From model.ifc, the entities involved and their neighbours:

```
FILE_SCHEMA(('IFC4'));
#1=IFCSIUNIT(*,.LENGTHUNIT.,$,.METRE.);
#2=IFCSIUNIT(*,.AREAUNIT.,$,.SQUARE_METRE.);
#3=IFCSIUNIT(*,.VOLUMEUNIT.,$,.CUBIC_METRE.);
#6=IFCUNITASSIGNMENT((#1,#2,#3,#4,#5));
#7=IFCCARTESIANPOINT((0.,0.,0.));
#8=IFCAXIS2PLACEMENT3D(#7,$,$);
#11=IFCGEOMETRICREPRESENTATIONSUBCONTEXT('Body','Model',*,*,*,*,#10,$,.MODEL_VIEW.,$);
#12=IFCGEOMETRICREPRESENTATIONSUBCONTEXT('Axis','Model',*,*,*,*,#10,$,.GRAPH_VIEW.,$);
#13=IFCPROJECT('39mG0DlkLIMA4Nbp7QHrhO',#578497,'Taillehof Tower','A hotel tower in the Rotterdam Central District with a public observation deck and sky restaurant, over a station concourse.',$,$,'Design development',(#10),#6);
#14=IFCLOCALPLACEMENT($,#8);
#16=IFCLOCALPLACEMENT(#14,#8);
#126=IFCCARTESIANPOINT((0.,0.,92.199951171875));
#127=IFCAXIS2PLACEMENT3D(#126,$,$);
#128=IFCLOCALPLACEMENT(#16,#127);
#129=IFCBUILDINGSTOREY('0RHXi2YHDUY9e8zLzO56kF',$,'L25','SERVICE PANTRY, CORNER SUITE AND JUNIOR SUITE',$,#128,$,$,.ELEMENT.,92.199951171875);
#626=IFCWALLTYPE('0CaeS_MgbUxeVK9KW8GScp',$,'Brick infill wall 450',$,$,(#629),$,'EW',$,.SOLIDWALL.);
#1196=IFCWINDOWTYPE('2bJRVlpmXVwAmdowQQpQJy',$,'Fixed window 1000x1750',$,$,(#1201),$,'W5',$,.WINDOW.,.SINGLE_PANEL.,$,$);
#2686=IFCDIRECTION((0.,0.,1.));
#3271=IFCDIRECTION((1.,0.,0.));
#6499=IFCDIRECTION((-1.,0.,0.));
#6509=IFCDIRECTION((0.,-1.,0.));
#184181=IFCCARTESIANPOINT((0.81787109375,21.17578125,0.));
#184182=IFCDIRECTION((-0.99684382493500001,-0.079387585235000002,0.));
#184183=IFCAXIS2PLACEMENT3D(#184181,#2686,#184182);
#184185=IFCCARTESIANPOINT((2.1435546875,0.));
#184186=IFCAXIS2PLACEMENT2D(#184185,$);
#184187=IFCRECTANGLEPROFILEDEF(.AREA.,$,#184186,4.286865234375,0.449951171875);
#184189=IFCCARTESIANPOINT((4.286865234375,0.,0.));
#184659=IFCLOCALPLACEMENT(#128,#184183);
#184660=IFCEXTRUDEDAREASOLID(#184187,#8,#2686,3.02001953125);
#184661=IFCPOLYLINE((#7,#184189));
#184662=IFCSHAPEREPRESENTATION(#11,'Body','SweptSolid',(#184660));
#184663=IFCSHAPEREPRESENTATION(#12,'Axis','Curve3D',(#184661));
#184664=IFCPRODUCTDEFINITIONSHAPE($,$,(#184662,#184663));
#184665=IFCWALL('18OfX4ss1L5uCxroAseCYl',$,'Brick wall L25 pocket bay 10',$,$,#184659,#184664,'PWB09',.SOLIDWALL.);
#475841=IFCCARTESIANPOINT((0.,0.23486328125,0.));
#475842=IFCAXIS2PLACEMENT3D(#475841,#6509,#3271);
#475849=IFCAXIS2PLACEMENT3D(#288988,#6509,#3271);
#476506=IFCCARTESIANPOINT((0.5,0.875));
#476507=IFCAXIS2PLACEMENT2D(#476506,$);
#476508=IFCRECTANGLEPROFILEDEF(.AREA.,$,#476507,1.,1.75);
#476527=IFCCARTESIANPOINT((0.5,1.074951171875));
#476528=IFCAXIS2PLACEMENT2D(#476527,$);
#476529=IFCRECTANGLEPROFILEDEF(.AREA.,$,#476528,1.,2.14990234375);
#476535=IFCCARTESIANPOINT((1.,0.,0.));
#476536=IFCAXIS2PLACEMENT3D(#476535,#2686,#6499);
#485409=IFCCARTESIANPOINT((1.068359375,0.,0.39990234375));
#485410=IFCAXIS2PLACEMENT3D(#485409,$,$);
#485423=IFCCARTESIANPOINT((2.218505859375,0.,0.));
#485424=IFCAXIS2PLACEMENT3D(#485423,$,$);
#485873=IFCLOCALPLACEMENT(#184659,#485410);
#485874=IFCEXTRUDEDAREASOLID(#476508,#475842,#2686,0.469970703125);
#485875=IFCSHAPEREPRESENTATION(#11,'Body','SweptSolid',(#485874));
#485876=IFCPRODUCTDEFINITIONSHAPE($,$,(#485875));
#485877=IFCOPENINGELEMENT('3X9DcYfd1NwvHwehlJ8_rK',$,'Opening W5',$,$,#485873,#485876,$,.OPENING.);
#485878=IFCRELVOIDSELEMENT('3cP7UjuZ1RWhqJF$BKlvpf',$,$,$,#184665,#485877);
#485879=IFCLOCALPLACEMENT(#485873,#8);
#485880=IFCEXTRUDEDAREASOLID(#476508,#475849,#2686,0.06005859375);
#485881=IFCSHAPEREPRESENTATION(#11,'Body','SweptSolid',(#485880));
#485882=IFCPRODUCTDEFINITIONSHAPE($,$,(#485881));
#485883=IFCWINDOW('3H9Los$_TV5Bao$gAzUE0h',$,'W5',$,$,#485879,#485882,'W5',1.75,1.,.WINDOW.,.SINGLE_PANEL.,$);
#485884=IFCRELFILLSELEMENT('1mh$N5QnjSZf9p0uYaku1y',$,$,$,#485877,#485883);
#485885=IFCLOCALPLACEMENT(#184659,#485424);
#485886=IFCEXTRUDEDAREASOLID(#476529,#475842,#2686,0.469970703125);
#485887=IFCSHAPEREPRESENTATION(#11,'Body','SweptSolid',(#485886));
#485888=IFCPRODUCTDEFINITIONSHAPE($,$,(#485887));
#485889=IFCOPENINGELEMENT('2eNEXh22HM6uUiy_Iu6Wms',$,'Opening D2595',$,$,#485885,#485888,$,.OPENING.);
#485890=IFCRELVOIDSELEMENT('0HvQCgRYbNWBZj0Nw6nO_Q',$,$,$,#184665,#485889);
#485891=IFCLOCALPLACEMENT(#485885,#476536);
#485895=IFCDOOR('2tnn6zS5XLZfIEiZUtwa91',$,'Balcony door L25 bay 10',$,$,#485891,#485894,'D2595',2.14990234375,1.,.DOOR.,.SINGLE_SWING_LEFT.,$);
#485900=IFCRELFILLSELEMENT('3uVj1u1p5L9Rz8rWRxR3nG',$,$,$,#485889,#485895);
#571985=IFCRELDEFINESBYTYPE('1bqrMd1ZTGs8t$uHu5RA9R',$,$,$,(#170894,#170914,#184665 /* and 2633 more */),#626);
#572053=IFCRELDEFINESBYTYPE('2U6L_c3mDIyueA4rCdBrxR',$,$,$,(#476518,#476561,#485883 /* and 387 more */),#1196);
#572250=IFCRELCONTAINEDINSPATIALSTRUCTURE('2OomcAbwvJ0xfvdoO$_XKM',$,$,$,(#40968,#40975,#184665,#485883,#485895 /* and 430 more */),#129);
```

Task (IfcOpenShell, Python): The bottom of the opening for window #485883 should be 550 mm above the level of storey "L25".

```python
import numpy as np
import ifcopenshell
import ifcopenshell.api.geometry
import ifcopenshell.geom
import ifcopenshell.util.element
import ifcopenshell.util.placement
import ifcopenshell.util.shape
import ifcopenshell.util.unit

model = ifcopenshell.open("model.ifc")
unit_scale = ifcopenshell.util.unit.calculate_unit_scale(model)

window = model.by_guid("3H9Los$_TV5Bao$gAzUE0h")
opening = window.FillsVoids[0].RelatingOpeningElement
storey = ifcopenshell.util.element.get_container(window, ifc_class="IfcBuildingStorey")
level = ifcopenshell.util.placement.get_local_placement(storey.ObjectPlacement)[2, 3]

# The opening's origin need not be at the sill, so measure its lowest point.
shape = ifcopenshell.geom.create_shape(ifcopenshell.geom.settings(), opening)
bottom = ifcopenshell.util.shape.get_shape_bottom_elevation(shape, shape.geometry) / unit_scale
dz = level + 0.55 / unit_scale - bottom

shift = np.array([0.0, 0.0, dz])
# The window is placed relative to its opening, so it follows when the opening moves.
matrix = ifcopenshell.util.placement.get_local_placement(opening.ObjectPlacement)
matrix[:3, 3] += shift
ifcopenshell.api.geometry.edit_object_placement(
    model, product=opening, matrix=matrix, is_si=False, should_transform_children=True
)

print(f"moved by {dz * unit_scale:+.3f} m")

model.write("model_updated.ifc")
```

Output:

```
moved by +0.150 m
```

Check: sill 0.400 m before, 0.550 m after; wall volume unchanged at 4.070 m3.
